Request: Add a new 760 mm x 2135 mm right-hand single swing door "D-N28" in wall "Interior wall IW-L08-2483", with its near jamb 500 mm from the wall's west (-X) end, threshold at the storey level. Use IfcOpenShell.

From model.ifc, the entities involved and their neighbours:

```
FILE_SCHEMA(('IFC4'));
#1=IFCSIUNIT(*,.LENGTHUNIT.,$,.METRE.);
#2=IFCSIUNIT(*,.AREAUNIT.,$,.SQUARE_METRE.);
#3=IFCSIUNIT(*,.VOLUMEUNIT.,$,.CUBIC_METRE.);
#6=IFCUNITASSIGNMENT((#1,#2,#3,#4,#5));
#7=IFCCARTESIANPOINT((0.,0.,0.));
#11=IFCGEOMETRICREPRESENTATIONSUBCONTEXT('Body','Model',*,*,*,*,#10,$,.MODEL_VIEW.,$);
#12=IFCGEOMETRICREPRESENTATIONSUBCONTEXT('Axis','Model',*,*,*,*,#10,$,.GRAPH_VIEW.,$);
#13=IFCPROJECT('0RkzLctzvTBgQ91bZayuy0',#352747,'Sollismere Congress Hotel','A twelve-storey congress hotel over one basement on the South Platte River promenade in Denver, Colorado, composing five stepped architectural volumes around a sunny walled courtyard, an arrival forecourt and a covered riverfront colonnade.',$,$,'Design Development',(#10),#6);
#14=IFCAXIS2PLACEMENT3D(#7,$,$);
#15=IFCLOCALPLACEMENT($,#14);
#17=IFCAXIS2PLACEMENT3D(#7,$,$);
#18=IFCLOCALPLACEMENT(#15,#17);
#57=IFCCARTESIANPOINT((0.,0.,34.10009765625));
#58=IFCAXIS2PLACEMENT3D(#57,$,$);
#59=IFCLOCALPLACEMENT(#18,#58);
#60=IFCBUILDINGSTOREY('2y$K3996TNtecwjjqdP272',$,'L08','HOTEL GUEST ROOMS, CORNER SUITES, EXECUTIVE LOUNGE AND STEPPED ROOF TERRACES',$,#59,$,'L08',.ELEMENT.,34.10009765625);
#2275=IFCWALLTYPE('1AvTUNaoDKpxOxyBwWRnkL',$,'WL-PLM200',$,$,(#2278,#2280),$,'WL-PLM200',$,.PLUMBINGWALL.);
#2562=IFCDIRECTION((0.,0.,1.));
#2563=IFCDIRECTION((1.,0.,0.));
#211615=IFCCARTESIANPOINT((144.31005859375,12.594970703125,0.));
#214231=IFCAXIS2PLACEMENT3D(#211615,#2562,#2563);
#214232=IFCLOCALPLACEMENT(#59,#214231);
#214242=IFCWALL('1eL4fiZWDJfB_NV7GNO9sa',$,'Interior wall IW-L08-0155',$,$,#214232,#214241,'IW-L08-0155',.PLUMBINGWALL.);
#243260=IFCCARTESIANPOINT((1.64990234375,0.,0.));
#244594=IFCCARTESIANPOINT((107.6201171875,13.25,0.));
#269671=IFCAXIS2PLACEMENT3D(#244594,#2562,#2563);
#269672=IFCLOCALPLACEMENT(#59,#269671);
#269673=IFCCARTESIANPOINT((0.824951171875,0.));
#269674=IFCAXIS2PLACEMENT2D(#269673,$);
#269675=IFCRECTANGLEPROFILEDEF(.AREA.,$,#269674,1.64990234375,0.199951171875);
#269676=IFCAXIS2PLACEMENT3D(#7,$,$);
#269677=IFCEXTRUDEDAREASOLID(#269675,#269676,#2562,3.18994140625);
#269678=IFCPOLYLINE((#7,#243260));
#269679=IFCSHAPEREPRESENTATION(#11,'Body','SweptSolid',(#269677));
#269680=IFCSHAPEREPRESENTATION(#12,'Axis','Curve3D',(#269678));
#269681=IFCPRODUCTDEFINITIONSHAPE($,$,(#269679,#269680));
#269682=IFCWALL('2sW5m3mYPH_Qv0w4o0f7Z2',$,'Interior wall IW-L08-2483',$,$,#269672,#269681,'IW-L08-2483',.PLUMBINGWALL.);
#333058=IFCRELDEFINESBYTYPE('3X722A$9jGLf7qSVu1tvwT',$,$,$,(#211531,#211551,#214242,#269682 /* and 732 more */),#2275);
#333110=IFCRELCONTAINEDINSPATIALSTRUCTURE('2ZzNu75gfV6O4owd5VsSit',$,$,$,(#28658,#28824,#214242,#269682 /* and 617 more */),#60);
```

```python
import numpy as np
import ifcopenshell
import ifcopenshell.api.feature
import ifcopenshell.api.geometry
import ifcopenshell.api.root
import ifcopenshell.api.spatial
import ifcopenshell.geom
import ifcopenshell.util.element
import ifcopenshell.util.placement
import ifcopenshell.util.representation
import ifcopenshell.util.shape
import ifcopenshell.util.unit

model = ifcopenshell.open("model.ifc")
unit_scale = ifcopenshell.util.unit.calculate_unit_scale(model)
settings = ifcopenshell.geom.settings()


def volume(element):
    """Net volume in cubic metres, openings subtracted."""
    shape = ifcopenshell.geom.create_shape(settings, element)
    return ifcopenshell.util.shape.get_volume(shape.geometry)


wall = model.by_id(269682)
storey = ifcopenshell.util.element.get_container(wall, ifc_class="IfcBuildingStorey")
context = ifcopenshell.util.representation.get_context(model, "Model", "Body", "MODEL_VIEW")
before = volume(wall)

width, height, from_end, sill = 0.76, 2.135, 0.5, 0.0  # metres

# The wall runs along its own X axis, and the end named is its -X end.
wall_shape = ifcopenshell.geom.create_shape(settings, wall)
x, y, z = ifcopenshell.util.shape.get_vertices(wall_shape.geometry).T
start = x.min() + from_end
face, thickness = float(y.min()), float(y.max() - y.min())
wall_matrix = ifcopenshell.util.placement.get_local_placement(wall.ObjectPlacement)
level = ifcopenshell.util.placement.get_local_placement(storey.ObjectPlacement)[2, 3]


def in_wall(x, y):
    """Placement at x, y metres in the wall's axes, at sill height."""
    matrix = wall_matrix.copy()
    matrix[:, 3] = wall_matrix @ np.array([x / unit_scale, y / unit_scale, 0.0, 1.0])
    matrix[2, 3] = level + sill / unit_scale
    return matrix


# Opening: a box that overshoots both wall faces by 50 mm.
opening = ifcopenshell.api.root.create_entity(model, ifc_class="IfcOpeningElement", predefined_type="OPENING")
box = ifcopenshell.api.geometry.add_wall_representation(
    model, context=context, length=width, height=height, thickness=thickness + 0.1
)
ifcopenshell.api.geometry.assign_representation(model, product=opening, representation=box)
ifcopenshell.api.geometry.edit_object_placement(model, product=opening, matrix=in_wall(start, face - 0.05), is_si=False)
ifcopenshell.api.feature.add_feature(model, feature=opening, element=wall)

door = ifcopenshell.api.root.create_entity(model, ifc_class="IfcDoor", name="D-N28", predefined_type="DOOR")
door.OverallWidth, door.OverallHeight = width / unit_scale, height / unit_scale
door.OperationType = "SINGLE_SWING_RIGHT"
body = ifcopenshell.api.geometry.add_door_representation(
    model,
    context=context,
    overall_width=door.OverallWidth,
    overall_height=door.OverallHeight,
    operation_type="SINGLE_SWING_RIGHT",
    lining_properties={"LiningDepth": thickness / unit_scale, "ThresholdDepth": thickness / unit_scale},
)
ifcopenshell.api.geometry.assign_representation(model, product=door, representation=body)
ifcopenshell.api.spatial.assign_container(model, products=[door], relating_structure=storey)
ifcopenshell.api.feature.add_filling(model, opening=opening, element=door)

# The lining spans the wall, so the door starts at the wall face.
ifcopenshell.api.geometry.edit_object_placement(model, product=door, matrix=in_wall(start, face), is_si=False)

after = volume(wall)

print(f"wall volume {before:.3f} -> {after:.3f} m3")

model.write("model-out.ifc")
```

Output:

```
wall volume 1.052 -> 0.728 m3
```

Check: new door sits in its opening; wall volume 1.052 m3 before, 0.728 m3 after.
